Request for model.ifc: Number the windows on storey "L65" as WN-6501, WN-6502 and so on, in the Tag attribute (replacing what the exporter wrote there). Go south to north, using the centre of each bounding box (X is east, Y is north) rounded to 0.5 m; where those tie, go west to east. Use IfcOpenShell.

First a look at what the model holds.

```python
import ifcopenshell
import ifcopenshell.util.element
import ifcopenshell.util.placement

model = ifcopenshell.open("model.ifc")
print(model.schema)
storey = next(s for s in model.by_type("IfcBuildingStorey") if s.Name == "L65")
windows = [e for e in ifcopenshell.util.element.get_decomposition(storey) if e.is_a("IfcWindow")]
for e in sorted(windows, key=lambda e: e.id()):
    origin = ifcopenshell.util.placement.get_local_placement(e.ObjectPlacement)[:3, 3]
    print(e.id(), e.Tag, e.Name, origin.round(2) + 0.0, sep=" | ")
```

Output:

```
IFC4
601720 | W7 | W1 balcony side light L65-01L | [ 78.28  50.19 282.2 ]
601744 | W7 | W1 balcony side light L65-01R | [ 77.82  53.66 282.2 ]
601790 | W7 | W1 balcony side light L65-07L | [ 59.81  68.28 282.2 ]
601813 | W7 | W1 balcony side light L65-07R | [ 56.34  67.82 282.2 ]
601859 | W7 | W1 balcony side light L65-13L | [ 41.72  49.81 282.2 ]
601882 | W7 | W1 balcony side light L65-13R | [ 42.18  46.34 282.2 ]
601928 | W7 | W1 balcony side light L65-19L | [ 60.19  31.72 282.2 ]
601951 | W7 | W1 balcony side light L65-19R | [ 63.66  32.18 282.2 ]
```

```python
import ifcopenshell
import ifcopenshell.geom
import ifcopenshell.util.element
import ifcopenshell.util.shape

model = ifcopenshell.open("model.ifc")
settings = ifcopenshell.geom.settings()
settings.set("use-world-coords", True)


def centre(element):
    shape = ifcopenshell.geom.create_shape(settings, element)
    return ifcopenshell.util.shape.get_bbox_centroid(shape.geometry)


storey = next(s for s in model.by_type("IfcBuildingStorey") if s.Name == "L65")
windows = [e for e in ifcopenshell.util.element.get_decomposition(storey) if e.is_a("IfcWindow")]

# Insertion points can sit at a corner or the storey origin, so sort by the geometry (in metres).
centres = {e: centre(e) for e in windows}
windows.sort(key=lambda e: (round(centres[e][1] / 0.5), centres[e][0]))

for i, e in enumerate(windows, start=1):
    number = f"WN-65{i:02d}"
    e.Tag = number
    print(e.id(), number)

model.write("model_rev.ifc")
```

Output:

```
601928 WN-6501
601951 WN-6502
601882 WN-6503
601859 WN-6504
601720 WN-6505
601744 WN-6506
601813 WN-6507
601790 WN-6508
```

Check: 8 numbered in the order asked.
